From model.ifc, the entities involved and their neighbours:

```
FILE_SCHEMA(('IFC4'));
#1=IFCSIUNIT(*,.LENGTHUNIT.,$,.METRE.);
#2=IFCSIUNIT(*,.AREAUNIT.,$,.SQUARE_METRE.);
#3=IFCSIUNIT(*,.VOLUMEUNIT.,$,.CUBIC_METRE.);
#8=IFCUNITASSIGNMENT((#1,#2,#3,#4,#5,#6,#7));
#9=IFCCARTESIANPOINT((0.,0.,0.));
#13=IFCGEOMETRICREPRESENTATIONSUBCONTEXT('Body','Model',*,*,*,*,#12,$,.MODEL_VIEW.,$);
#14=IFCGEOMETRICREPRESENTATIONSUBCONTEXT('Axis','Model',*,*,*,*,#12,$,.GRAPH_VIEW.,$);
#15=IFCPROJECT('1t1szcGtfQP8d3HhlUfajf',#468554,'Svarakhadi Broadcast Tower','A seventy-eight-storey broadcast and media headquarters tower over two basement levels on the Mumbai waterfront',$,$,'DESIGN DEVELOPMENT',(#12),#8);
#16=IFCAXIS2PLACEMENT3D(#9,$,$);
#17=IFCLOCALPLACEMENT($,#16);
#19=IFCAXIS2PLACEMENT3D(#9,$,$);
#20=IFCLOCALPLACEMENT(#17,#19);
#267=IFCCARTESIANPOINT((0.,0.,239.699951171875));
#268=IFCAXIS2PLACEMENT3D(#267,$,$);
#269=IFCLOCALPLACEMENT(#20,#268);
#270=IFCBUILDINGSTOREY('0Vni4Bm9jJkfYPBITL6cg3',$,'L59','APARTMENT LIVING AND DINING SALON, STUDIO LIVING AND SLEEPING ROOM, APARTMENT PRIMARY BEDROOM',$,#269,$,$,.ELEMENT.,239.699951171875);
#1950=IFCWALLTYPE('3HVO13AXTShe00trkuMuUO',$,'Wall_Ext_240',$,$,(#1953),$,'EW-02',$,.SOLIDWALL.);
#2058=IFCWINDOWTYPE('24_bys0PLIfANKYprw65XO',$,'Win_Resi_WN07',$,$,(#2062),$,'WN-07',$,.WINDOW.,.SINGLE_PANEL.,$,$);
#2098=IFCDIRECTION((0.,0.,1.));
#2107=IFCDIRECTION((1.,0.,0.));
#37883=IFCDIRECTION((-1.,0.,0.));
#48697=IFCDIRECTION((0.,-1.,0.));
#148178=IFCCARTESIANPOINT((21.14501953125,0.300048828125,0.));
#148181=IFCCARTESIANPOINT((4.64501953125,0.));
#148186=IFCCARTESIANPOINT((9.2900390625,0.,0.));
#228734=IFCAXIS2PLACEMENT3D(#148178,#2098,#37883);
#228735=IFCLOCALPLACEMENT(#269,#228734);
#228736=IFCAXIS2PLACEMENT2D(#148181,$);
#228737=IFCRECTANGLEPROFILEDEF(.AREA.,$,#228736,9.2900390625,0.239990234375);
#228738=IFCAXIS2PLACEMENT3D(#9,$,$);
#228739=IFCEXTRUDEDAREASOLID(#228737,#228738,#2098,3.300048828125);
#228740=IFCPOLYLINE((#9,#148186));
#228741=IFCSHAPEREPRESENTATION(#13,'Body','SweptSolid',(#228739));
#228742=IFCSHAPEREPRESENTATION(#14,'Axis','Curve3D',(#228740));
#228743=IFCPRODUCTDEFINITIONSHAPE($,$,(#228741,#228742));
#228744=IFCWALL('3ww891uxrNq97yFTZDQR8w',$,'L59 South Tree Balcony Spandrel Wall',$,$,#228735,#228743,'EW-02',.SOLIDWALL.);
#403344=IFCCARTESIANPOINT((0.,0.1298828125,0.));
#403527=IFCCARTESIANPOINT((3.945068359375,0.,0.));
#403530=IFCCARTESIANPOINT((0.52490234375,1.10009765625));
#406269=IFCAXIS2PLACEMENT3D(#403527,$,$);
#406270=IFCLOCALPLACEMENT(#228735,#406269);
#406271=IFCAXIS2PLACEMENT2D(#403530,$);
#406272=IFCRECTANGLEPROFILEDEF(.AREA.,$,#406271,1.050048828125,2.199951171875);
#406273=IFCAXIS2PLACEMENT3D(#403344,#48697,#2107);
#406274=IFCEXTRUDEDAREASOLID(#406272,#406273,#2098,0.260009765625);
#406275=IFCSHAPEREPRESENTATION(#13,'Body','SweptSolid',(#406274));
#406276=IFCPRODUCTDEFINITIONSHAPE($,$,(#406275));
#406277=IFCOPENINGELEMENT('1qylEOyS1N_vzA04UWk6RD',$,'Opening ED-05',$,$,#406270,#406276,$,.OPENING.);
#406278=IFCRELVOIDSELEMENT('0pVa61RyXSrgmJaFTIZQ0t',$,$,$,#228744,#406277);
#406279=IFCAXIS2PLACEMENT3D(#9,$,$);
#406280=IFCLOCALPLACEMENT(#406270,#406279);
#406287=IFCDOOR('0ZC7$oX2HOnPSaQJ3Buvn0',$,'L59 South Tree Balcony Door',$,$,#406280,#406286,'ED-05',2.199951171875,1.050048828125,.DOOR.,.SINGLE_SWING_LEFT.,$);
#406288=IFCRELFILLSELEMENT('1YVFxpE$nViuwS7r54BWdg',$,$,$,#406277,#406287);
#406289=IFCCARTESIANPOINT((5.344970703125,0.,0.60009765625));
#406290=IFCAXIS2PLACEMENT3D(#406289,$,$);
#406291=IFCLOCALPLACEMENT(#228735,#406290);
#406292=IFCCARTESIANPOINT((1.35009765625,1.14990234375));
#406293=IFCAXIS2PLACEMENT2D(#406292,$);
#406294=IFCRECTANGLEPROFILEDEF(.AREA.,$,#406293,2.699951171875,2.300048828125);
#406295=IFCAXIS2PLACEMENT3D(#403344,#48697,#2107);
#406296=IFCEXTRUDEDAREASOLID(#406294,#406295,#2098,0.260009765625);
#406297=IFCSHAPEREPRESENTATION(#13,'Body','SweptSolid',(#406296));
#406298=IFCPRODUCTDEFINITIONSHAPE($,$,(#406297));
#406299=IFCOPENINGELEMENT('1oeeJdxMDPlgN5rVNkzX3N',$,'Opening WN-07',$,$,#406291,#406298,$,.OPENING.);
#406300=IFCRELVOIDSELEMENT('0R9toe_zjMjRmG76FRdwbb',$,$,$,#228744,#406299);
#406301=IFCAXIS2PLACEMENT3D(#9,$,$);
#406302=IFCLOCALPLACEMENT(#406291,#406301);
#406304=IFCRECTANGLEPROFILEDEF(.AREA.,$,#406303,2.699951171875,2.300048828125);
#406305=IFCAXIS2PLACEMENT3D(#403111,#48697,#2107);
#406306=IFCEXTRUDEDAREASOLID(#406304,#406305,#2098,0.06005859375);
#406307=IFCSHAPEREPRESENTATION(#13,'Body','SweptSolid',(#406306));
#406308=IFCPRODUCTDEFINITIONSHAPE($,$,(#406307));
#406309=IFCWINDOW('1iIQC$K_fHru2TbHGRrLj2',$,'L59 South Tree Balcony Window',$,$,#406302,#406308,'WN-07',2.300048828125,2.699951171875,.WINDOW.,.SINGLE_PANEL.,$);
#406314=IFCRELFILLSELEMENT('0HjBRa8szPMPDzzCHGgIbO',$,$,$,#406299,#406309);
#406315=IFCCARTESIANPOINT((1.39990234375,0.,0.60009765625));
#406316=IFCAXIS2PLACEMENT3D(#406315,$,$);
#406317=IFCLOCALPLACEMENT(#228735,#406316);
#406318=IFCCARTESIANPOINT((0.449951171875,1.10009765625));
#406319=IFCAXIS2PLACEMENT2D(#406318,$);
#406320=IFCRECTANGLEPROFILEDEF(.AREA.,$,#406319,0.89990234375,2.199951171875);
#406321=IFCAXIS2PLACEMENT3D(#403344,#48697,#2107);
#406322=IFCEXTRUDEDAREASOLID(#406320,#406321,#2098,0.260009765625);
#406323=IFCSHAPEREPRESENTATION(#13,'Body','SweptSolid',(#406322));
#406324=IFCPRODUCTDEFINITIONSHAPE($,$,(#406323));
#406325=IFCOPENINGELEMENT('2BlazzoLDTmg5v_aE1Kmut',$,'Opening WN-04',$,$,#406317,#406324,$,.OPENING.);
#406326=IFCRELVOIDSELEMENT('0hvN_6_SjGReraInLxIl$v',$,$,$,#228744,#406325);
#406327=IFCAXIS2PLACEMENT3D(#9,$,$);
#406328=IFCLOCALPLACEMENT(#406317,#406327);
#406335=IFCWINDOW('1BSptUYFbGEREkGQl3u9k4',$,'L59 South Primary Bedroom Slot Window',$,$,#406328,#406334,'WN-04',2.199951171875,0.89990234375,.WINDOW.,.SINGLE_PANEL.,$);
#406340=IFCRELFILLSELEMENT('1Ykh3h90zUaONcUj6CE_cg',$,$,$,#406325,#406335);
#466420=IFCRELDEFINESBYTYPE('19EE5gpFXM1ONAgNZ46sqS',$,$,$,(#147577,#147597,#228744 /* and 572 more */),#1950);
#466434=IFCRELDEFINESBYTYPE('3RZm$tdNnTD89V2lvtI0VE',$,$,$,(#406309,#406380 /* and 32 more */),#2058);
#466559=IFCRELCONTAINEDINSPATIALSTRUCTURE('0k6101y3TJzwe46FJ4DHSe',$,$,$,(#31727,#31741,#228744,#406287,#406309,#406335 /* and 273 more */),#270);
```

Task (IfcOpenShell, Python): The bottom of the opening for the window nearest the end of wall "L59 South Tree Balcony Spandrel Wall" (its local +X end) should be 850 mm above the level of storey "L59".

```python
import numpy as np
import ifcopenshell
import ifcopenshell.api.geometry
import ifcopenshell.geom
import ifcopenshell.util.element
import ifcopenshell.util.placement
import ifcopenshell.util.shape
import ifcopenshell.util.unit

model = ifcopenshell.open("model.ifc")
unit_scale = ifcopenshell.util.unit.calculate_unit_scale(model)

window = model.by_guid("1iIQC$K_fHru2TbHGRrLj2")
opening = window.FillsVoids[0].RelatingOpeningElement
storey = ifcopenshell.util.element.get_container(window, ifc_class="IfcBuildingStorey")
level = ifcopenshell.util.placement.get_local_placement(storey.ObjectPlacement)[2, 3]

# The opening's origin need not be at the sill, so measure its lowest point.
shape = ifcopenshell.geom.create_shape(ifcopenshell.geom.settings(), opening)
bottom = ifcopenshell.util.shape.get_shape_bottom_elevation(shape, shape.geometry) / unit_scale
dz = level + 0.85 - bottom

shift = np.array([0.0, 0.0, dz])
# The window is placed relative to its opening, so it follows when the opening moves.
matrix = ifcopenshell.util.placement.get_local_placement(opening.ObjectPlacement)
matrix[:3, 3] += shift
ifcopenshell.api.geometry.edit_object_placement(
    model, product=opening, matrix=matrix, is_si=False, should_transform_children=True
)

print(f"moved by {dz * unit_scale:+.3f} m")

model.write("model_rev.ifc")
```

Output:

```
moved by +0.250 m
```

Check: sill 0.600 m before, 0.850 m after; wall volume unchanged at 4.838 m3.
